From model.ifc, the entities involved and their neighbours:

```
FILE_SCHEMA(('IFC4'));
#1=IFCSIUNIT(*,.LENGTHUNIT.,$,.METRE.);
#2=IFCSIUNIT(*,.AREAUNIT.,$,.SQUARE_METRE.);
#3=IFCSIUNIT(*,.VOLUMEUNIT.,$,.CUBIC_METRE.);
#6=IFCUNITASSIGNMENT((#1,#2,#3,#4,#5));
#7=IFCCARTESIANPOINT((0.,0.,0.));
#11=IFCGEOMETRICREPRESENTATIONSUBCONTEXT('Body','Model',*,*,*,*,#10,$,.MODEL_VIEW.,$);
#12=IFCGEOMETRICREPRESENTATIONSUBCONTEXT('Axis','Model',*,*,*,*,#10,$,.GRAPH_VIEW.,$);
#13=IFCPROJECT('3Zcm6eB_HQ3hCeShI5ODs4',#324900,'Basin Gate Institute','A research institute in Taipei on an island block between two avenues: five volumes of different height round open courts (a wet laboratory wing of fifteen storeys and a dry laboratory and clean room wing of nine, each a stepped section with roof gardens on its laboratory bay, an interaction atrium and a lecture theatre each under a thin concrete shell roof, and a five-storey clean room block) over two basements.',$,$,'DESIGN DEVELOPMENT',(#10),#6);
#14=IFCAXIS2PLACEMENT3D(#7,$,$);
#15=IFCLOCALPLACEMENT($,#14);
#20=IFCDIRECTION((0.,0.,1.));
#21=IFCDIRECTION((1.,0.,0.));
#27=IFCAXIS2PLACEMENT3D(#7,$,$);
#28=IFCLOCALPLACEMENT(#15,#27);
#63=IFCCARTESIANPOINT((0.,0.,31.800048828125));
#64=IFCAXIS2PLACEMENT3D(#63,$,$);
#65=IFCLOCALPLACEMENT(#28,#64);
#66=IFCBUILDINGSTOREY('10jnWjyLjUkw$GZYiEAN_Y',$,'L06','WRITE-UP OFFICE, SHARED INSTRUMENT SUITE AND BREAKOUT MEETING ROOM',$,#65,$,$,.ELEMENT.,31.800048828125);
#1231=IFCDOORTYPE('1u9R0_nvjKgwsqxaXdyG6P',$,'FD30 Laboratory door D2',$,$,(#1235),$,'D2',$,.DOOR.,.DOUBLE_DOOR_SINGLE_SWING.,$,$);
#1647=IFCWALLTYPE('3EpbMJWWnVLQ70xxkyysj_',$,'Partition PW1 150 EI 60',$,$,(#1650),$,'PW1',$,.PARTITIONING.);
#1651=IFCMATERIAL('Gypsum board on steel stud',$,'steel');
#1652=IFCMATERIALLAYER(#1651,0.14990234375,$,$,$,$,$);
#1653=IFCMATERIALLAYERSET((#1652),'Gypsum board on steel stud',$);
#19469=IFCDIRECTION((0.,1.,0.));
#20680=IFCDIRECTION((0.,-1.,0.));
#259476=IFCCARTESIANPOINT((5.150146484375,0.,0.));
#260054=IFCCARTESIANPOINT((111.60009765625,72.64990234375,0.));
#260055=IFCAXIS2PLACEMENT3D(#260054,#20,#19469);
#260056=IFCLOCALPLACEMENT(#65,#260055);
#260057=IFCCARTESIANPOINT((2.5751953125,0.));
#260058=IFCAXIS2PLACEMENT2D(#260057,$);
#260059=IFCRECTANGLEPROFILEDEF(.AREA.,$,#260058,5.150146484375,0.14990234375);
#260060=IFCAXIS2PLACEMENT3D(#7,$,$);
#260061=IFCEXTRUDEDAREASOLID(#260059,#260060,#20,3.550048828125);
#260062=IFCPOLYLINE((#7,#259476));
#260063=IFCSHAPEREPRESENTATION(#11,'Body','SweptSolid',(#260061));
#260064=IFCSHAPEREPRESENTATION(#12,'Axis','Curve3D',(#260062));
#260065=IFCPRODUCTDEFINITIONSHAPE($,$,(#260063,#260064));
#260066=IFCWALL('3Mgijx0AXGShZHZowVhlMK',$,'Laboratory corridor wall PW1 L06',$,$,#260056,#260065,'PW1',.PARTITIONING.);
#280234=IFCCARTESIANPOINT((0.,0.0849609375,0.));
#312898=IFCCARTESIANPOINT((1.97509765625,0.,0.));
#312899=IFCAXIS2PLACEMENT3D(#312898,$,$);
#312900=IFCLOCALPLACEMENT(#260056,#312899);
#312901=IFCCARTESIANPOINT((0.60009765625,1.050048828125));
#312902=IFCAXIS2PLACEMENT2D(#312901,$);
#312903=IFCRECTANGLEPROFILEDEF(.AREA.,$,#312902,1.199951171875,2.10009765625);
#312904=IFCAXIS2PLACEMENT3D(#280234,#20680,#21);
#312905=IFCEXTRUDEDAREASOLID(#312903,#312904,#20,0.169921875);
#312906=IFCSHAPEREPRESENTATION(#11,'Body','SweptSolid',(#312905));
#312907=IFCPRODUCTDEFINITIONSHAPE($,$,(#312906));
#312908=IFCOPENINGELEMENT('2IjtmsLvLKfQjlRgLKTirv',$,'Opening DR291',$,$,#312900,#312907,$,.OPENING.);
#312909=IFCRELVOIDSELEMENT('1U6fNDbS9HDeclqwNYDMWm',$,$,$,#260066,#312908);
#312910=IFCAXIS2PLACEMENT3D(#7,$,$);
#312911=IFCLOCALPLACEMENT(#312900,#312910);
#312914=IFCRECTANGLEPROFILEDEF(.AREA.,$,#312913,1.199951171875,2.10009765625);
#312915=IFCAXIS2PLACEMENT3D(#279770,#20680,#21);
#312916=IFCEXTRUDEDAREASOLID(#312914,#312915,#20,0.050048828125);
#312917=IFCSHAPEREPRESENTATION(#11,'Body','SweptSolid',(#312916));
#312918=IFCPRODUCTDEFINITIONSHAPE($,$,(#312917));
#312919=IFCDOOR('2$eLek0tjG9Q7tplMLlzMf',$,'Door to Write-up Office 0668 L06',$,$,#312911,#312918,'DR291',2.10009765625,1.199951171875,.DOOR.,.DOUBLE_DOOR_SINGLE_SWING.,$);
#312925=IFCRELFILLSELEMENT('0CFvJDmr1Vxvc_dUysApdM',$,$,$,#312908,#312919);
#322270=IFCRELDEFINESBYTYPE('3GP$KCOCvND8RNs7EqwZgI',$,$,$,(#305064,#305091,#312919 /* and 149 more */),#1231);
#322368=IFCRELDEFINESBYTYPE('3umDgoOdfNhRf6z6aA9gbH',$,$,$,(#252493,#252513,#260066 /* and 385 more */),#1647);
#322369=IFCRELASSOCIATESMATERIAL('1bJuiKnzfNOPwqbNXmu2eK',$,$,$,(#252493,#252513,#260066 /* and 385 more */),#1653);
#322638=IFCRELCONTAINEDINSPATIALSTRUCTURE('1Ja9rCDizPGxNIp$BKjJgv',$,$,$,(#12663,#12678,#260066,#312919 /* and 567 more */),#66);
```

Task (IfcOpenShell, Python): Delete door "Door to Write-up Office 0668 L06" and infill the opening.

```python
import ifcopenshell
import ifcopenshell.api.feature
import ifcopenshell.api.root
import ifcopenshell.geom
import ifcopenshell.util.shape

model = ifcopenshell.open("model.ifc")
settings = ifcopenshell.geom.settings()


def volume(element):
    """Net volume in cubic metres, openings subtracted."""
    shape = ifcopenshell.geom.create_shape(settings, element)
    return ifcopenshell.util.shape.get_volume(shape.geometry)


door = model.by_id(312919)
opening = door.FillsVoids[0].RelatingOpeningElement
wall = opening.VoidsElements[0].RelatingBuildingElement
before = volume(wall)

ifcopenshell.api.root.remove_product(model, product=door)
ifcopenshell.api.feature.remove_feature(model, feature=opening)

after = volume(wall)

print(f"wall volume {before:.3f} -> {after:.3f} m3")

model.write("model_rev.ifc")
```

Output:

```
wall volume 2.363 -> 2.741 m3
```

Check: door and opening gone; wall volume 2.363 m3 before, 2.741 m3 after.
